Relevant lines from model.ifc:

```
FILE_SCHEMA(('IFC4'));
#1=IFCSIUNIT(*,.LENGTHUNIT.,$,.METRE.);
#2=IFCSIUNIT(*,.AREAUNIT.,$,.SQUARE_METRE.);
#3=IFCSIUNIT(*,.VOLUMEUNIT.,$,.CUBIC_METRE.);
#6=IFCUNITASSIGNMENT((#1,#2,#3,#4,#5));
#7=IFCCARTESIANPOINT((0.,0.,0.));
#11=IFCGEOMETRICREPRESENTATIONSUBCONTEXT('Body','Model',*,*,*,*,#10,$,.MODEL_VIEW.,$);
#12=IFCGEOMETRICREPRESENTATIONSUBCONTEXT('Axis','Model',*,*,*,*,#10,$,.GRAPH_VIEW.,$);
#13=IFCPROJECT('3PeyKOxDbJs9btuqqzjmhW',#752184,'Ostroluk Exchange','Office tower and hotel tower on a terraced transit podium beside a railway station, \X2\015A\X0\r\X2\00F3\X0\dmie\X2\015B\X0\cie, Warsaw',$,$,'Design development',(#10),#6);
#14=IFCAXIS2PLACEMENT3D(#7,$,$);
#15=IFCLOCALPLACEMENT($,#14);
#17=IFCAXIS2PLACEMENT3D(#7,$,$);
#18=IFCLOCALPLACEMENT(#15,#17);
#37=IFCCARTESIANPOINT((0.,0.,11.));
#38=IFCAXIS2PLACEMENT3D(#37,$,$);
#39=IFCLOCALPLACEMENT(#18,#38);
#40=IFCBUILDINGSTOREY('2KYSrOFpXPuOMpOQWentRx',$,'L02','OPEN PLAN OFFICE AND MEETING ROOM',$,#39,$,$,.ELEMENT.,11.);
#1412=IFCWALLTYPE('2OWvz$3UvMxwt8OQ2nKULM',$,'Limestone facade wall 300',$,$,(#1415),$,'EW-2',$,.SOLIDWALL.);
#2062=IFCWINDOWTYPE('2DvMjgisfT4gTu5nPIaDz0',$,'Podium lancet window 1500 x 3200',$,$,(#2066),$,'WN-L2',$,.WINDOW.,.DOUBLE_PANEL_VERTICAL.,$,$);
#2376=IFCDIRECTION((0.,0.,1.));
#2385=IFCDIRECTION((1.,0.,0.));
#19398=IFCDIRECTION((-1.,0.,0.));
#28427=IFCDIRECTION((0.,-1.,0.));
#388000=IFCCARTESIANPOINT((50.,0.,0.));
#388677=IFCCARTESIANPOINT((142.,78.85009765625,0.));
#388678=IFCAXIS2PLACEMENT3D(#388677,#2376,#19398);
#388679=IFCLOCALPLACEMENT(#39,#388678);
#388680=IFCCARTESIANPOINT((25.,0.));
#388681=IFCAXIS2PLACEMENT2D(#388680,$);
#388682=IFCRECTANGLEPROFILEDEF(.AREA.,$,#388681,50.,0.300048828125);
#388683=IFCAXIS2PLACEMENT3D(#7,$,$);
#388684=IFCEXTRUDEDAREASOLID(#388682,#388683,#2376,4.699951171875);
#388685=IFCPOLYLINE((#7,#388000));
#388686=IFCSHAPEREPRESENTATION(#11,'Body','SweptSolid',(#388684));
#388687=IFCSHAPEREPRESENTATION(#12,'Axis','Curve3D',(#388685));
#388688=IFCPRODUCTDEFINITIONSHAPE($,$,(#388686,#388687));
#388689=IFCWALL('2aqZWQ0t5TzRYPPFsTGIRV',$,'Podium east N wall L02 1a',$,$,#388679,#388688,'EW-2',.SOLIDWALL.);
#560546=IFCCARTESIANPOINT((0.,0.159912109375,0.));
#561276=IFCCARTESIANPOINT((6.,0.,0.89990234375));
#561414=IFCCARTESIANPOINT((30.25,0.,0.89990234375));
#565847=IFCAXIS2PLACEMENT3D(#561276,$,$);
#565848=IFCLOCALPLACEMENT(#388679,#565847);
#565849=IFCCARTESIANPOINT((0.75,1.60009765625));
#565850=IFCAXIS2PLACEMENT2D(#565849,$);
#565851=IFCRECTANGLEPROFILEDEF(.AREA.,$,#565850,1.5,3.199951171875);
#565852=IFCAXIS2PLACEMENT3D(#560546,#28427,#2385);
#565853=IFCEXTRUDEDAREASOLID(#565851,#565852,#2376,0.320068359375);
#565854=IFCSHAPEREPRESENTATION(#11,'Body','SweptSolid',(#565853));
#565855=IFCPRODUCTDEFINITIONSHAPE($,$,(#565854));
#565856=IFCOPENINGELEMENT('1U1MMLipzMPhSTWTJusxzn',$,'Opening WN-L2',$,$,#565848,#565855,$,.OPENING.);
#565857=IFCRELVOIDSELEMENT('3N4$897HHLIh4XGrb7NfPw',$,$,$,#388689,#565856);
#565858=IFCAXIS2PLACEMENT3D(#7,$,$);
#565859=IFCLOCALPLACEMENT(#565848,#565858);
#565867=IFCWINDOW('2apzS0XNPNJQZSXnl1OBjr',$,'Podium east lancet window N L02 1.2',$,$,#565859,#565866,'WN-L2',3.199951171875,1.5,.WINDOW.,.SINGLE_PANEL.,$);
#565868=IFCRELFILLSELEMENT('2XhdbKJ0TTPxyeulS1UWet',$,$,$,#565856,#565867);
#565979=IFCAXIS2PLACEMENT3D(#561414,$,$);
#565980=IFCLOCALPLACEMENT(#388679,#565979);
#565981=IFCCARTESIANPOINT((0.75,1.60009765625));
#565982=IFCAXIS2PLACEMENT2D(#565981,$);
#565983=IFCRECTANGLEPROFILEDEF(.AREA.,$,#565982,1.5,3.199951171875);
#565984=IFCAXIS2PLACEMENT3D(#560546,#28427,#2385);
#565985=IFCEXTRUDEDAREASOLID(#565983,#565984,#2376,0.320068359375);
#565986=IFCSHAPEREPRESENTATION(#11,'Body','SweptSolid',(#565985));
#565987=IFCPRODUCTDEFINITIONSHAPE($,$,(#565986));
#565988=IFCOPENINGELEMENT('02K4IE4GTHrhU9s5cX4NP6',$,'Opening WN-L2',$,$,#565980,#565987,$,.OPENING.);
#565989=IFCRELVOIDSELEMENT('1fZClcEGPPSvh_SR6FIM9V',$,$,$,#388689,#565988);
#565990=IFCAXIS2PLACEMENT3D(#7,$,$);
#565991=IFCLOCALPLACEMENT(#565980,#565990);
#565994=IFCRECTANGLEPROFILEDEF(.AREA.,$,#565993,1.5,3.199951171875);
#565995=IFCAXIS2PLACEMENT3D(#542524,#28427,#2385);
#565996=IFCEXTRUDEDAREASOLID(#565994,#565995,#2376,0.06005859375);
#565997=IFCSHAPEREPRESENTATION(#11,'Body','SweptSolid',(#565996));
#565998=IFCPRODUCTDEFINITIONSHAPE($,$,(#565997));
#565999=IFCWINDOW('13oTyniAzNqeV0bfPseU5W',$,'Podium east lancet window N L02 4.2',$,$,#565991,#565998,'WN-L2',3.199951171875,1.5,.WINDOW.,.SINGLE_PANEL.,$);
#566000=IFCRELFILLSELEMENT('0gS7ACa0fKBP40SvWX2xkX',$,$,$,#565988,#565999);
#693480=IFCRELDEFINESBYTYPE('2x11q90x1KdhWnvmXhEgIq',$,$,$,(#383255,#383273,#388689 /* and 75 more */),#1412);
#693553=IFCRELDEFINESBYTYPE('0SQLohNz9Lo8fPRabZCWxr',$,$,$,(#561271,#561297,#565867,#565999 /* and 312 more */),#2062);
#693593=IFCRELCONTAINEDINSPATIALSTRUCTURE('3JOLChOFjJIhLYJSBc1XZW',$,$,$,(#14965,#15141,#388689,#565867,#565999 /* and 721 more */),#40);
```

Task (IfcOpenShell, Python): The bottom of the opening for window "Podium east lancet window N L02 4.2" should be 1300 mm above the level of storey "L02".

```python
import numpy as np
import ifcopenshell
import ifcopenshell.api.geometry
import ifcopenshell.geom
import ifcopenshell.util.element
import ifcopenshell.util.placement
import ifcopenshell.util.shape
import ifcopenshell.util.unit

model = ifcopenshell.open("model.ifc")
unit_scale = ifcopenshell.util.unit.calculate_unit_scale(model)

window = model.by_guid("13oTyniAzNqeV0bfPseU5W")
opening = window.FillsVoids[0].RelatingOpeningElement
storey = ifcopenshell.util.element.get_container(window, ifc_class="IfcBuildingStorey")
level = ifcopenshell.util.placement.get_local_placement(storey.ObjectPlacement)[2, 3]

# The opening's origin need not be at the sill, so measure its lowest point.
shape = ifcopenshell.geom.create_shape(ifcopenshell.geom.settings(), opening)
bottom = ifcopenshell.util.shape.get_shape_bottom_elevation(shape, shape.geometry) / unit_scale
dz = level + 1.3 - bottom

shift = np.array([0.0, 0.0, dz])
# The window is placed relative to its opening, so it follows when the opening moves.
matrix = ifcopenshell.util.placement.get_local_placement(opening.ObjectPlacement)
matrix[:3, 3] += shift
ifcopenshell.api.geometry.edit_object_placement(
    model, product=opening, matrix=matrix, is_si=False, should_transform_children=True
)

print(f"moved by {dz * unit_scale:+.3f} m")

model.write("model_rev.ifc")
```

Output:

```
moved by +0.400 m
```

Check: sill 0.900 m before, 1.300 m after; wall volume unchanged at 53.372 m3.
